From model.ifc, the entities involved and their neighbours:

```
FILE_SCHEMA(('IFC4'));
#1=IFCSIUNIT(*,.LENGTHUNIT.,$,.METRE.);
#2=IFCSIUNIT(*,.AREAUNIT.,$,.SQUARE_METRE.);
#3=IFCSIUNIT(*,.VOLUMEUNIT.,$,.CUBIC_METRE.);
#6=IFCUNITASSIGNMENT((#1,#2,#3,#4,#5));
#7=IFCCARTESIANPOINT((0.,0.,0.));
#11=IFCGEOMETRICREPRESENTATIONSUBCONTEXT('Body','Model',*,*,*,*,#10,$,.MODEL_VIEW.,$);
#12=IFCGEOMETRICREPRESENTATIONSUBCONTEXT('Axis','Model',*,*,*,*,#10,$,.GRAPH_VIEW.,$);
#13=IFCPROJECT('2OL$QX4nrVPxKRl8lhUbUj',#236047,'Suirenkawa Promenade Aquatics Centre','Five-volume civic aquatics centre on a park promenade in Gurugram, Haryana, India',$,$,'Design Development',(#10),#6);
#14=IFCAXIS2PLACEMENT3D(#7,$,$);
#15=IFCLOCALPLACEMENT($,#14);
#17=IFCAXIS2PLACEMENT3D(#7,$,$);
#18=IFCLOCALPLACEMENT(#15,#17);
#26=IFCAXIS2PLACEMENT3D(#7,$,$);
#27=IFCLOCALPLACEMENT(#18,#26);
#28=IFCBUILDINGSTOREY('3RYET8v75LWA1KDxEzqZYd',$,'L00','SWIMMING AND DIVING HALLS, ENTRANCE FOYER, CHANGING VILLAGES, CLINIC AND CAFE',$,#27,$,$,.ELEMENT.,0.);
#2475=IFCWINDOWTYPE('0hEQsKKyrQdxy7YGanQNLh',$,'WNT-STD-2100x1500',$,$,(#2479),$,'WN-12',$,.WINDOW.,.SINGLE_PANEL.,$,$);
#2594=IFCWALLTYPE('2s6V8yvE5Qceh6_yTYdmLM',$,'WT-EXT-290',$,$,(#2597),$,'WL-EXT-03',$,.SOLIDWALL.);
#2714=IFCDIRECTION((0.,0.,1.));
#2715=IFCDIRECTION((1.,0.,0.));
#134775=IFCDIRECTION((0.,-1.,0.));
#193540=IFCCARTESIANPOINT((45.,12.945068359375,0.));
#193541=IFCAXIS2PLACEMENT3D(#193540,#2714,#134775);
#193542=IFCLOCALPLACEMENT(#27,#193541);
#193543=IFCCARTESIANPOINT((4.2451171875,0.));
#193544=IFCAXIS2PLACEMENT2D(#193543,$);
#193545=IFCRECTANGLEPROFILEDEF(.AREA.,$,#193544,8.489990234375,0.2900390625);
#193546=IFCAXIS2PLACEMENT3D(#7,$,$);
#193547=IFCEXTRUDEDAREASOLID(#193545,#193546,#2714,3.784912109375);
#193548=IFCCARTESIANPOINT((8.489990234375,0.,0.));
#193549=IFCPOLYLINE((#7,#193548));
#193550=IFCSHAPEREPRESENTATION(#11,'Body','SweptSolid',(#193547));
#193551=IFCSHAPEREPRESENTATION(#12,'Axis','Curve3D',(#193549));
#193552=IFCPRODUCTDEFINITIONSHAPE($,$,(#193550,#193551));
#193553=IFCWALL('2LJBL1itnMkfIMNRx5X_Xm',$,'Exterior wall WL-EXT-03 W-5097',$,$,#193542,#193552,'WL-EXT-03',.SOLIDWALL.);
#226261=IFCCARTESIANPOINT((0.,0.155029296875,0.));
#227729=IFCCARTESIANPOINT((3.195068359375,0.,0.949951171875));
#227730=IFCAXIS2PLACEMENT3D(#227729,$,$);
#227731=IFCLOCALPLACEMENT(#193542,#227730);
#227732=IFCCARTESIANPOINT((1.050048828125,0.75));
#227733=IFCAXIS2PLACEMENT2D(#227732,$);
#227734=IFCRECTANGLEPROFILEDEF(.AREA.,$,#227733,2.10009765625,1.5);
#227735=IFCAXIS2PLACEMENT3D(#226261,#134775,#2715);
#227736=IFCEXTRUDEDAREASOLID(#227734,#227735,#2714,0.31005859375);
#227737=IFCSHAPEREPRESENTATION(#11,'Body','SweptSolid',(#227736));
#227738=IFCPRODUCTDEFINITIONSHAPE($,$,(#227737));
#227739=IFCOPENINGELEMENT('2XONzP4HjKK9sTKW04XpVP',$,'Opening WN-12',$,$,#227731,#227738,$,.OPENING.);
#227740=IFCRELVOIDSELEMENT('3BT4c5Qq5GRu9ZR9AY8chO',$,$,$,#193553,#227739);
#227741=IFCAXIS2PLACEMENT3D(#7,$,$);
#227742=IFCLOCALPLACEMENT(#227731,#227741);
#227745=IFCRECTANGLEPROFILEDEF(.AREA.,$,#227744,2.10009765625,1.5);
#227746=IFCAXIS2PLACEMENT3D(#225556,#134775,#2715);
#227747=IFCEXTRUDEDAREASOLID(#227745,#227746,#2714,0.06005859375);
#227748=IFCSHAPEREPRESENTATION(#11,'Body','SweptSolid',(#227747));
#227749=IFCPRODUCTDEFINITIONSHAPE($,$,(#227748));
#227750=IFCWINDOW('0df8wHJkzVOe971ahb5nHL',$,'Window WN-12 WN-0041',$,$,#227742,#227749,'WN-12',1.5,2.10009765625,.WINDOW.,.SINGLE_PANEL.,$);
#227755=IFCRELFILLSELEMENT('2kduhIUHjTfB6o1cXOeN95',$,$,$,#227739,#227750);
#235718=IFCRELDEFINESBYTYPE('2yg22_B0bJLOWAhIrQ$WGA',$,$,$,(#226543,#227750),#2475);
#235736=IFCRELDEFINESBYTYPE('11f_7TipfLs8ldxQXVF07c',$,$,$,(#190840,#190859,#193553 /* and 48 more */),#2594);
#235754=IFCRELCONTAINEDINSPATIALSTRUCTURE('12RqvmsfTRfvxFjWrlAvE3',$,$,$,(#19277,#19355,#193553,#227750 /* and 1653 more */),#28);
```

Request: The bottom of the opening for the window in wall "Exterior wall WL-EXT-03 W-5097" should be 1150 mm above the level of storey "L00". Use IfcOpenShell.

```python
import numpy as np
import ifcopenshell
import ifcopenshell.api.geometry
import ifcopenshell.geom
import ifcopenshell.util.element
import ifcopenshell.util.placement
import ifcopenshell.util.shape
import ifcopenshell.util.unit

model = ifcopenshell.open("model.ifc")
unit_scale = ifcopenshell.util.unit.calculate_unit_scale(model)

window = model.by_guid("0df8wHJkzVOe971ahb5nHL")
opening = window.FillsVoids[0].RelatingOpeningElement
storey = ifcopenshell.util.element.get_container(window, ifc_class="IfcBuildingStorey")
level = ifcopenshell.util.placement.get_local_placement(storey.ObjectPlacement)[2, 3]

# The opening's origin need not be at the sill, so measure its lowest point.
shape = ifcopenshell.geom.create_shape(ifcopenshell.geom.settings(), opening)
bottom = ifcopenshell.util.shape.get_shape_bottom_elevation(shape, shape.geometry) / unit_scale
dz = level + 1.15 / unit_scale - bottom

shift = np.array([0.0, 0.0, dz])
# The window is placed relative to its opening, so it follows when the opening moves.
matrix = ifcopenshell.util.placement.get_local_placement(opening.ObjectPlacement)
matrix[:3, 3] += shift
ifcopenshell.api.geometry.edit_object_placement(
    model, product=opening, matrix=matrix, is_si=False, should_transform_children=True
)

print(f"moved by {dz * unit_scale:+.3f} m")

model.write("model_rev.ifc")
```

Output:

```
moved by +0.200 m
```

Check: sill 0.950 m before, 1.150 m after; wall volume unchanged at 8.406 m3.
